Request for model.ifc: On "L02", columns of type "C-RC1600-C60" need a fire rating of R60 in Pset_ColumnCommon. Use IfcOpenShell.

First a look at what the model holds.

```python
import ifcopenshell
import ifcopenshell.util.element

model = ifcopenshell.open("model.ifc")
print(model.schema)
storey = next(s for s in model.by_type("IfcBuildingStorey") if s.Name == "L02")
columns = [e for e in ifcopenshell.util.element.get_decomposition(storey) if e.is_a("IfcColumn")]
seen = {}
for e in columns:
    element_type = ifcopenshell.util.element.get_type(e)
    key = (element_type.Name if element_type != e and element_type else None, ifcopenshell.util.element.get_pset(e, "Pset_ColumnCommon", "FireRating"))
    seen[key] = seen.get(key, 0) + 1
for (name, value), count in sorted(seen.items(), key=str):
    print(count, "x", name, "|", value)
```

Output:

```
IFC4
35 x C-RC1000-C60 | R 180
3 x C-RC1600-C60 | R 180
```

```python
import ifcopenshell
import ifcopenshell.api.pset
import ifcopenshell.util.element

model = ifcopenshell.open("model.ifc")

storey = next(s for s in model.by_type("IfcBuildingStorey") if s.Name == "L02")
columns = [e for e in ifcopenshell.util.element.get_decomposition(storey) if e.is_a("IfcColumn")]

count = 0
for e in columns:
    element_type = ifcopenshell.util.element.get_type(e)
    if element_type in (None, e) or element_type.Name != "C-RC1600-C60":
        continue
    found = ifcopenshell.util.element.get_pset(e, "Pset_ColumnCommon", should_inherit=False)
    if found:
        pset = model.by_id(found["id"])
        if len(ifcopenshell.util.element.get_elements_by_pset(pset)) > 1:
            pset = ifcopenshell.api.pset.unshare_pset(model, products=[e], pset=pset)[0]
    else:
        pset = ifcopenshell.api.pset.add_pset(model, product=e, name="Pset_ColumnCommon")
    ifcopenshell.api.pset.edit_pset(model, pset=pset, properties={"FireRating": "R60"})
    count += 1

print(count, "columns updated")

model.write("model_v2.ifc")
```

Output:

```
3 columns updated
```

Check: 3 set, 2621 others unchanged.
